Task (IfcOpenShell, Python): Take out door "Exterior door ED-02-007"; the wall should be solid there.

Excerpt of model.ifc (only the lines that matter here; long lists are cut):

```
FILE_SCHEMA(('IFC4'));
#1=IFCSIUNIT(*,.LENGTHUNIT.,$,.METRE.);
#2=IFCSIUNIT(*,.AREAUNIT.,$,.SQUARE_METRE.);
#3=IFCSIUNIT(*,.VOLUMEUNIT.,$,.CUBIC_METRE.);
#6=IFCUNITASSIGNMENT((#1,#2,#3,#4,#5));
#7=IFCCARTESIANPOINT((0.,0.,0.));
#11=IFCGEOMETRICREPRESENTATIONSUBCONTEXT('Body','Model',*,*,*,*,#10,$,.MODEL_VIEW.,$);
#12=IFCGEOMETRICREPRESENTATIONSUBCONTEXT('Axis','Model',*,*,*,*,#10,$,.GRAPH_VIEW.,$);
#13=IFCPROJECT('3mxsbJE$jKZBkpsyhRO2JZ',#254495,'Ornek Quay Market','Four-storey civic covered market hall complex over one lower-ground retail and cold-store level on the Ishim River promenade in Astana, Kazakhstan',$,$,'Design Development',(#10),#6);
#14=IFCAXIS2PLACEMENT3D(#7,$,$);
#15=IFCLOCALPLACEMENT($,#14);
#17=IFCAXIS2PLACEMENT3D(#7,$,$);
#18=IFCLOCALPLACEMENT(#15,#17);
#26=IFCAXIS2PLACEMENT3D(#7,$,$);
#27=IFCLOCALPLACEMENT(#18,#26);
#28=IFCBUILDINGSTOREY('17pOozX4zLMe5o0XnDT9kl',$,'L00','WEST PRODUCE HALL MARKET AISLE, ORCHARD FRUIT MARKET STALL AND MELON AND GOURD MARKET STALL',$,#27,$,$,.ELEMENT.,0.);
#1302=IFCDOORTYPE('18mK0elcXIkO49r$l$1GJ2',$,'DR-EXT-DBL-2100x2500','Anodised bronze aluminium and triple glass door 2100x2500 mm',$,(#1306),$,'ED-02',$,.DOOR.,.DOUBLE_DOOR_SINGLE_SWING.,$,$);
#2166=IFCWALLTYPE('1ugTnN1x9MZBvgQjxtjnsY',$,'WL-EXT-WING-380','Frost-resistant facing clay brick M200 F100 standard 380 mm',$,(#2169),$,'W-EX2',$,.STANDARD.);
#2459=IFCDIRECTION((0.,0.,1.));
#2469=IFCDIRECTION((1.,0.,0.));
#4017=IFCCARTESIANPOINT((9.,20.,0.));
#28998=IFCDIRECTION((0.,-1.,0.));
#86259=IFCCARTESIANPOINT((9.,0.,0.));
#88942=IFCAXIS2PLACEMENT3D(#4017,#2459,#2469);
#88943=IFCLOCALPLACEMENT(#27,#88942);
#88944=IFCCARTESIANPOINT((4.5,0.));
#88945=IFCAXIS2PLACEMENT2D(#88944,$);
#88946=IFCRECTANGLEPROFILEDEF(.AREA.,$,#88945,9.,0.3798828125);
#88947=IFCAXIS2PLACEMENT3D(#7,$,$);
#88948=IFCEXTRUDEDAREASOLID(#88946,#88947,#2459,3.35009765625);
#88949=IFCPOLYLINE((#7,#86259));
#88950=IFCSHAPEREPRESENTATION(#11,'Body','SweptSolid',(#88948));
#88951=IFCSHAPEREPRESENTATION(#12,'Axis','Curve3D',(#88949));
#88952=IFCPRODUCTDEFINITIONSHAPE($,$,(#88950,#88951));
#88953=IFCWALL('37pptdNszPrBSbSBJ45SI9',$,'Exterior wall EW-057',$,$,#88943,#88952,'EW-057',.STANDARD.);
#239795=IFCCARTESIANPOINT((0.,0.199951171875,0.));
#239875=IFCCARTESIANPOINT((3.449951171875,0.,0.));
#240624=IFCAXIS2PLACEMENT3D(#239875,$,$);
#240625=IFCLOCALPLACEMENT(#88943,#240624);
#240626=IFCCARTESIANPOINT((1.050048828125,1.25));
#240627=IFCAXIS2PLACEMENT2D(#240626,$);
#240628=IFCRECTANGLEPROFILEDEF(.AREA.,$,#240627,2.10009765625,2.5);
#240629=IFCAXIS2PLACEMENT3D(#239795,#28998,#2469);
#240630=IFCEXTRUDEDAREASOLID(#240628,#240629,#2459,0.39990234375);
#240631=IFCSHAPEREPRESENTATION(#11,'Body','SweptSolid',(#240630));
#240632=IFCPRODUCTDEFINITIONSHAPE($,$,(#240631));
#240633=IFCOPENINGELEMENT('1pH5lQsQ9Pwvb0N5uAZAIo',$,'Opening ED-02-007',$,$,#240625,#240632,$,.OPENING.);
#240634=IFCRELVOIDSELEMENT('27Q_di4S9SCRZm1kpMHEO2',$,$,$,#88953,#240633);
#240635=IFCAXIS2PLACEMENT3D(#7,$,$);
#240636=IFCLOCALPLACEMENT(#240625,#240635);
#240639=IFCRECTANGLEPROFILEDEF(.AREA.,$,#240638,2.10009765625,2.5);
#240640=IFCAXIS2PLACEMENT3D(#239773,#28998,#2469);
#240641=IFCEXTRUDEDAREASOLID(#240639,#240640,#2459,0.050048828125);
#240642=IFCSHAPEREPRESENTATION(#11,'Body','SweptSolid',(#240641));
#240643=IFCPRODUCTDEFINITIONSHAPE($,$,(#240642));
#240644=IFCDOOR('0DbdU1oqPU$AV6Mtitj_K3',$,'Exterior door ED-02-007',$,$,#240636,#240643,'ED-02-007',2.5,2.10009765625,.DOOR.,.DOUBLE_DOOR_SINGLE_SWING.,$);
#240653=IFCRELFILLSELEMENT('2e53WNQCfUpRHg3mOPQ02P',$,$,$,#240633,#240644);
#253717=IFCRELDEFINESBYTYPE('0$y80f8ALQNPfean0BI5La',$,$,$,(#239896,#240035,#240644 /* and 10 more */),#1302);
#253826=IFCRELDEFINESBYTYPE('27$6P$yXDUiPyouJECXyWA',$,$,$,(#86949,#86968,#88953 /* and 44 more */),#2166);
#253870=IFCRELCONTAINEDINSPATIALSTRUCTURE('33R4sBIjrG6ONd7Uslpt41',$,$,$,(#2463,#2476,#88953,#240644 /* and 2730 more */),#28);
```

```python
import ifcopenshell
import ifcopenshell.api.feature
import ifcopenshell.api.root
import ifcopenshell.geom
import ifcopenshell.util.shape

model = ifcopenshell.open("model.ifc")
settings = ifcopenshell.geom.settings()


def volume(element):
    """Net volume in cubic metres, openings subtracted."""
    shape = ifcopenshell.geom.create_shape(settings, element)
    return ifcopenshell.util.shape.get_volume(shape.geometry)


door = model.by_guid("0DbdU1oqPU$AV6Mtitj_K3")
opening = door.FillsVoids[0].RelatingOpeningElement
wall = opening.VoidsElements[0].RelatingBuildingElement
before = volume(wall)

ifcopenshell.api.root.remove_product(model, product=door)
ifcopenshell.api.feature.remove_feature(model, feature=opening)

after = volume(wall)

print(f"wall volume {before:.3f} -> {after:.3f} m3")

model.write("model_edited.ifc")
```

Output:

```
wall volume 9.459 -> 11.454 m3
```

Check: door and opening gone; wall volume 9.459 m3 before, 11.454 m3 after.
